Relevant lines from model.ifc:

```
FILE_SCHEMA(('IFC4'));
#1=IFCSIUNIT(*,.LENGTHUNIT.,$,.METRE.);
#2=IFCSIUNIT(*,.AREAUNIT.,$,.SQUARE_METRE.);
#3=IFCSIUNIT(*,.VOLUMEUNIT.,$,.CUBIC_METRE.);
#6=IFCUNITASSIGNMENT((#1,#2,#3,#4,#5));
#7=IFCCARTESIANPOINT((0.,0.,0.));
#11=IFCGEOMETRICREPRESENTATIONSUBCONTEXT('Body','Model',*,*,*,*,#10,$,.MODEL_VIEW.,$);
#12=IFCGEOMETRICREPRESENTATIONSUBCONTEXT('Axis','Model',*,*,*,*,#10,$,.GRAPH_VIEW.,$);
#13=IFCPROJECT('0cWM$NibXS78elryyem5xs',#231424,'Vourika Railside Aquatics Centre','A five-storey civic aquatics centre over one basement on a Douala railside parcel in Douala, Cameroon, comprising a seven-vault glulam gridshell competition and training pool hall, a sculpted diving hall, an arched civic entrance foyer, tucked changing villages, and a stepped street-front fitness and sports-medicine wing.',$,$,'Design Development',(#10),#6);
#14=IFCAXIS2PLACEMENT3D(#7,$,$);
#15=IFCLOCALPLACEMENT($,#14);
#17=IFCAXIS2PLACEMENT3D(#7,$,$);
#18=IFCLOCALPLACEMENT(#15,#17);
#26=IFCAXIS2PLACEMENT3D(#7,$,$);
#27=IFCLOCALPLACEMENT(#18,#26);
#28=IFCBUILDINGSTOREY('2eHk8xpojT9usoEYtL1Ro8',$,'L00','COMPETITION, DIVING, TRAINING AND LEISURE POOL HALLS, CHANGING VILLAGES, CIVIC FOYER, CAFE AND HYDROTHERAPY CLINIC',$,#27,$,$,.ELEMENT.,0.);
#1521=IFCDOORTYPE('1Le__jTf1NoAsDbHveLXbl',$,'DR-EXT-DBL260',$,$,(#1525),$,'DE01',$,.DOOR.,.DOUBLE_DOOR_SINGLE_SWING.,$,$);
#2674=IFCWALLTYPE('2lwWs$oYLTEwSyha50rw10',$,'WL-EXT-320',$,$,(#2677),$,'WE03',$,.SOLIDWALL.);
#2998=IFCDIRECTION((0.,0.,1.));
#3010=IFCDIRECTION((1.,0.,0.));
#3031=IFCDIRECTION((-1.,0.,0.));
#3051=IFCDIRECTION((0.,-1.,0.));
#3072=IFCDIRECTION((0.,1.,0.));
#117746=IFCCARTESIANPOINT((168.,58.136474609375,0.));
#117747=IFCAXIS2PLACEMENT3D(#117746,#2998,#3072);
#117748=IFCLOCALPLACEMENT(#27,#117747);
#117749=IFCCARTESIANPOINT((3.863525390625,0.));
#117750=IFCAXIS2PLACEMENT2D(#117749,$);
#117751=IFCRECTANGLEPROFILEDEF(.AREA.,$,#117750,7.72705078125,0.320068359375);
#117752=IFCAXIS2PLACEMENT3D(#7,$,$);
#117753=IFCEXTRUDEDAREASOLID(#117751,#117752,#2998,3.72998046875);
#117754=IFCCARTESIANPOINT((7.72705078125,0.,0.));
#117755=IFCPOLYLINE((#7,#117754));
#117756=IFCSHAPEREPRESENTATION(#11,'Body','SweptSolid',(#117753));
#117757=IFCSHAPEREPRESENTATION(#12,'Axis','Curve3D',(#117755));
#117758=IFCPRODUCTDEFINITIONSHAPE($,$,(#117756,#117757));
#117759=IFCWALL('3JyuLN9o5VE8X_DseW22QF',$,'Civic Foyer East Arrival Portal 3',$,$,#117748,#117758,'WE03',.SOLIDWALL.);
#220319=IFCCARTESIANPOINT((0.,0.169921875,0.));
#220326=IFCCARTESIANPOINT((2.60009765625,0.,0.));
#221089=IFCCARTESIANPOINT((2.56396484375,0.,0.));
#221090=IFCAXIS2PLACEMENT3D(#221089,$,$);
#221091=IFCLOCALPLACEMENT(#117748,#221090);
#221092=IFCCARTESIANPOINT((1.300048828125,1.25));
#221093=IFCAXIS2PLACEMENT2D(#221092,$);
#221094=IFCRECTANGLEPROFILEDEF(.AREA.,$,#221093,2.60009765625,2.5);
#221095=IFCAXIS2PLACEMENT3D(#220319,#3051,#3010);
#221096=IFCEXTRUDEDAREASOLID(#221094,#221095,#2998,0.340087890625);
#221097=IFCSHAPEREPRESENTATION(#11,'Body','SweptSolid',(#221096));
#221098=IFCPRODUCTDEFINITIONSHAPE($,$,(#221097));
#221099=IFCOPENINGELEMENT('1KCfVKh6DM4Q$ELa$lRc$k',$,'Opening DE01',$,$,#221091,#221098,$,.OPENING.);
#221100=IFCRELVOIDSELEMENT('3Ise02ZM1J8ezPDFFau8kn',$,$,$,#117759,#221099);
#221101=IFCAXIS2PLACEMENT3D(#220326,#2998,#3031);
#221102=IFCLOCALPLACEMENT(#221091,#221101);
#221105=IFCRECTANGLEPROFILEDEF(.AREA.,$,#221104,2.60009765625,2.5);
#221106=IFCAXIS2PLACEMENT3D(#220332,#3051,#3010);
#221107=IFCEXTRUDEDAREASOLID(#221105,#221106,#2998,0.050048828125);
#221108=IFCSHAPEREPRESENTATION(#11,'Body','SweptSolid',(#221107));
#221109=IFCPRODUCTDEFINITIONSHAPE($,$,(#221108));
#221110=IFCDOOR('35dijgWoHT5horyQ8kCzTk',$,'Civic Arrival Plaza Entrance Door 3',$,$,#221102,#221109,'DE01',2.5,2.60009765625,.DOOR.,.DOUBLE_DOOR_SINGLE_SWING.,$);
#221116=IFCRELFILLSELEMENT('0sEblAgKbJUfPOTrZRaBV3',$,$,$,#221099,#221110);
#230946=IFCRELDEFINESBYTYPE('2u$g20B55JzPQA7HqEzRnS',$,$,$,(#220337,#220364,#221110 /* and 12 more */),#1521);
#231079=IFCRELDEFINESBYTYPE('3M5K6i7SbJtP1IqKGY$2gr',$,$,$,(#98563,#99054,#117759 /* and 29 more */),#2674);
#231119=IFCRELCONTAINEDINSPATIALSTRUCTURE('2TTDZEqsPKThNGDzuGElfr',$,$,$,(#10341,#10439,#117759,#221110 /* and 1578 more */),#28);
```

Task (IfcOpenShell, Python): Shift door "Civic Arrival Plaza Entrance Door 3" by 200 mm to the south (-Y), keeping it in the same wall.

```python
import ifcopenshell
import ifcopenshell.api.geometry
import ifcopenshell.util.placement
import ifcopenshell.util.unit

model = ifcopenshell.open("model.ifc")
unit_scale = ifcopenshell.util.unit.calculate_unit_scale(model)

door = model.by_guid("35dijgWoHT5horyQ8kCzTk")
opening = door.FillsVoids[0].RelatingOpeningElement
wall = opening.VoidsElements[0].RelatingBuildingElement

wall_matrix = ifcopenshell.util.placement.get_local_placement(wall.ObjectPlacement)
shift = wall_matrix[:3, 0] * -0.2 / unit_scale
before = ifcopenshell.util.placement.get_local_placement(door.ObjectPlacement)[:3, 3].copy()

# The door is placed relative to its opening, so it follows when the opening moves.
matrix = ifcopenshell.util.placement.get_local_placement(opening.ObjectPlacement)
matrix[:3, 3] += shift
ifcopenshell.api.geometry.edit_object_placement(
    model, product=opening, matrix=matrix, is_si=False, should_transform_children=True
)

after = ifcopenshell.util.placement.get_local_placement(door.ObjectPlacement)[:3, 3]
print("door moved by", (after - before).round(3) + 0.0)

model.write("model_edited.ifc")
```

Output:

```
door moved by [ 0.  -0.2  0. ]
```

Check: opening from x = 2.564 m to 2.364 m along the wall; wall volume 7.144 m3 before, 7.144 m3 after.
